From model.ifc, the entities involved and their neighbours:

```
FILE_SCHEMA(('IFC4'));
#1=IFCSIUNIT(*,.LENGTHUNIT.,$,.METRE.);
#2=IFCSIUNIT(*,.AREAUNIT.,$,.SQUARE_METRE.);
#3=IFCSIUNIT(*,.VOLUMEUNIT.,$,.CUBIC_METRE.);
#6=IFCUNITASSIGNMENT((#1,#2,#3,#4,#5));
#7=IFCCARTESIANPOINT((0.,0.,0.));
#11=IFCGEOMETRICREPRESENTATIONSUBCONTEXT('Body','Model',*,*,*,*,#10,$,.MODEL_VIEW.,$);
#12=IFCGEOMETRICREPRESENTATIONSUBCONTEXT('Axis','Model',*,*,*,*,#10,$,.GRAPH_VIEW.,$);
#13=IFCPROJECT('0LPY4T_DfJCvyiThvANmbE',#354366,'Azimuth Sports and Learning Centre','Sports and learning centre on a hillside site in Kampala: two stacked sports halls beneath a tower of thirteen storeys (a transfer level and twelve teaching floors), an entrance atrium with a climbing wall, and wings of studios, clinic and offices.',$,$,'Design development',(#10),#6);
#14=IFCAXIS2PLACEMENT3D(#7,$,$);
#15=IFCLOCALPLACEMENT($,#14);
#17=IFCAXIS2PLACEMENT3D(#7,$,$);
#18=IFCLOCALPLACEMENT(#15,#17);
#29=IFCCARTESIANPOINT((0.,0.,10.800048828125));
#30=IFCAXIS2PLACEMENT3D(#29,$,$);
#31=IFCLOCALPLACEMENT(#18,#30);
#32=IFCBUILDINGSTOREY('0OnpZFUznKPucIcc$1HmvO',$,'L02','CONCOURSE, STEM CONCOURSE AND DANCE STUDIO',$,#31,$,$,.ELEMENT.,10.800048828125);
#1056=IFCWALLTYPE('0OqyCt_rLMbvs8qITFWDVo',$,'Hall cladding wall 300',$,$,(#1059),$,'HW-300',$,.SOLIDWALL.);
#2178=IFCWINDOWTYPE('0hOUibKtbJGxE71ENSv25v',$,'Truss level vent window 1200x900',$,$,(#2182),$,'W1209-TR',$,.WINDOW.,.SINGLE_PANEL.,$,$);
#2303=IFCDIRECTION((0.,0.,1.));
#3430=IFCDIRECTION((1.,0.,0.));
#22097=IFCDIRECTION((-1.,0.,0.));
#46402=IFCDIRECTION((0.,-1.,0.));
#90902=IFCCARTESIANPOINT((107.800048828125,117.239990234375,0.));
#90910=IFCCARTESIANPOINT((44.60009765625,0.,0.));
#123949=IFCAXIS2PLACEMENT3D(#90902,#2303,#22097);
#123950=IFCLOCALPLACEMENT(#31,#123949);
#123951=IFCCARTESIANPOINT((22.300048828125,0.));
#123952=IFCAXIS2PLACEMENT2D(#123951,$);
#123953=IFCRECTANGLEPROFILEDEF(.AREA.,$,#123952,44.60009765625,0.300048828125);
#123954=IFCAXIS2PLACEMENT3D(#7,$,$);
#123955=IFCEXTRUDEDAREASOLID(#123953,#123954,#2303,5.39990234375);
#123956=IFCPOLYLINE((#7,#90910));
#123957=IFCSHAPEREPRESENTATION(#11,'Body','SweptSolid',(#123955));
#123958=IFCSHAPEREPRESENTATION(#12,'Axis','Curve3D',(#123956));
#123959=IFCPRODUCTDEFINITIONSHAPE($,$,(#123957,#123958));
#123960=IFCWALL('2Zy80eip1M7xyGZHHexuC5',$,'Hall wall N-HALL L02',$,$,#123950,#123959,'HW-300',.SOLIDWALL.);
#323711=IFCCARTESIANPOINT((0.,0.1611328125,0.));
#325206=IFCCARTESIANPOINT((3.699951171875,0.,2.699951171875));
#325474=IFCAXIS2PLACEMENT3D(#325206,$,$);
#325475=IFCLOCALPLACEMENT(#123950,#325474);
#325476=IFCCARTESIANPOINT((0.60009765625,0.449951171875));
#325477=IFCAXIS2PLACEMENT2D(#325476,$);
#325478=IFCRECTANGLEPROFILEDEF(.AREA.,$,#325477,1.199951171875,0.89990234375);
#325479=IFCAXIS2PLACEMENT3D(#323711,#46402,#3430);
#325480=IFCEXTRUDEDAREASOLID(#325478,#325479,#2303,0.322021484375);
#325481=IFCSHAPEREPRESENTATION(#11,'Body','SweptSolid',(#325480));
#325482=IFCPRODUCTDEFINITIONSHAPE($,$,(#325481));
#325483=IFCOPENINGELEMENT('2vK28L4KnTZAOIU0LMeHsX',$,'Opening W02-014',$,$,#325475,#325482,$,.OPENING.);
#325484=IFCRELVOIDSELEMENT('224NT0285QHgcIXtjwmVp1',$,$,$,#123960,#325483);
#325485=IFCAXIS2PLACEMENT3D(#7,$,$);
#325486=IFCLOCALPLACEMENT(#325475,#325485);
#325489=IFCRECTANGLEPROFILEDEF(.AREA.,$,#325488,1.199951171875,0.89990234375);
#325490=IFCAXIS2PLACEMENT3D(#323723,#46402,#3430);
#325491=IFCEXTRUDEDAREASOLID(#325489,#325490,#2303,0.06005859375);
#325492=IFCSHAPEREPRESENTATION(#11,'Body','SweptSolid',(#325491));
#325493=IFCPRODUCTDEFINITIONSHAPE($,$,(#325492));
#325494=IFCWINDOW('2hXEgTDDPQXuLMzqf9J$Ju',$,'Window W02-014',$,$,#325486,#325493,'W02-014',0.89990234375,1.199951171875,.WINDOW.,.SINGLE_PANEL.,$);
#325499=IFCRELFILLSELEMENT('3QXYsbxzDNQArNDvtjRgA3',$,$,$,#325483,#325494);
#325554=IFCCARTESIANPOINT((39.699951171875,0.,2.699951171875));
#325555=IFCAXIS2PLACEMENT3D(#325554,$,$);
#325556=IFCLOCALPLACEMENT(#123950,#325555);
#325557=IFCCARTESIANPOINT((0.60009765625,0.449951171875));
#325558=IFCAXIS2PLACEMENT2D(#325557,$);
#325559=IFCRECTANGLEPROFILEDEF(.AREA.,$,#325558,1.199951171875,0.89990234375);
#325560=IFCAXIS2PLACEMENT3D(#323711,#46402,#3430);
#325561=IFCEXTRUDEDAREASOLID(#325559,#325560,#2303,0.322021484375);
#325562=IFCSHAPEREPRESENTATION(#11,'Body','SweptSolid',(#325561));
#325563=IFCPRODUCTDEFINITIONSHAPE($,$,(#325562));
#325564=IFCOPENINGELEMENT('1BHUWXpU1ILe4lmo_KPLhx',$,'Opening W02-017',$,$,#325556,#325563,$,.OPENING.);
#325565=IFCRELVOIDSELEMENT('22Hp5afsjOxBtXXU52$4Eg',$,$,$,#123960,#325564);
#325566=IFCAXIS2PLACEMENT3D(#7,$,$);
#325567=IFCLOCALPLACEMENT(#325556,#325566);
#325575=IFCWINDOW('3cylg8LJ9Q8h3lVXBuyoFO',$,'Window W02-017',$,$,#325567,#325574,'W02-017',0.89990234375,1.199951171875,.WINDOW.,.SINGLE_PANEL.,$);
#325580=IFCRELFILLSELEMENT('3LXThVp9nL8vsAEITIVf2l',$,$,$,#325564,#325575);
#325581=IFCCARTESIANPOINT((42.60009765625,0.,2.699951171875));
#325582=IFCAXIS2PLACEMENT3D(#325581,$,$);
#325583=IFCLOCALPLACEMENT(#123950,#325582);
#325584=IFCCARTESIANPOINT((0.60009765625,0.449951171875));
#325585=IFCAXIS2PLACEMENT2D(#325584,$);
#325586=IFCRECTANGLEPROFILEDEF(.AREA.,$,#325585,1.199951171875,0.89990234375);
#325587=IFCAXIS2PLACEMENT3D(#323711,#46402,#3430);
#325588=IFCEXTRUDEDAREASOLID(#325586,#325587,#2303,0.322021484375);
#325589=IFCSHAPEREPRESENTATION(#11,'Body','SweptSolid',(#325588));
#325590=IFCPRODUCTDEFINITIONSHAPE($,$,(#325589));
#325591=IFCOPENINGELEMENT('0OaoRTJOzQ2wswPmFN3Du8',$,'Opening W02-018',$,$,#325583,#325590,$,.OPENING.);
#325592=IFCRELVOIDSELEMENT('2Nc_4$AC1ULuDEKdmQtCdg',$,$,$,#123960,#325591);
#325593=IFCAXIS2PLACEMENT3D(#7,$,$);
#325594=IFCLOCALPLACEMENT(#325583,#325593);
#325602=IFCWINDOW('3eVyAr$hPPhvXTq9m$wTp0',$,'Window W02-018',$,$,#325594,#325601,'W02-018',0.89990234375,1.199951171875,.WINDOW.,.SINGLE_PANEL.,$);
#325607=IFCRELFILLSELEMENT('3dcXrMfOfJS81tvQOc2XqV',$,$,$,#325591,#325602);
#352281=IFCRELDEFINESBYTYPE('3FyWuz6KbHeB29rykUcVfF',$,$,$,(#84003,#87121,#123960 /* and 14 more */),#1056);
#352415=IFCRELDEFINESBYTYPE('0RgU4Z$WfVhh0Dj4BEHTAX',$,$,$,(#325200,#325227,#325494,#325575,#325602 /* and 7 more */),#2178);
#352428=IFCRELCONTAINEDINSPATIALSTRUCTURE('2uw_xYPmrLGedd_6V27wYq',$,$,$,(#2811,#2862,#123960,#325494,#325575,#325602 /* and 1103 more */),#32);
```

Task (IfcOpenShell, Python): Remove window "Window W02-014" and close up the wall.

```python
import ifcopenshell
import ifcopenshell.api.feature
import ifcopenshell.api.root
import ifcopenshell.geom
import ifcopenshell.util.shape

model = ifcopenshell.open("model.ifc")
settings = ifcopenshell.geom.settings()


def volume(element):
    """Net volume in cubic metres, openings subtracted."""
    shape = ifcopenshell.geom.create_shape(settings, element)
    return ifcopenshell.util.shape.get_volume(shape.geometry)


window = model.by_guid("2hXEgTDDPQXuLMzqf9J$Ju")
opening = window.FillsVoids[0].RelatingOpeningElement
wall = opening.VoidsElements[0].RelatingBuildingElement
before = volume(wall)

ifcopenshell.api.root.remove_product(model, product=window)
ifcopenshell.api.feature.remove_feature(model, feature=opening)

after = volume(wall)

print(f"wall volume {before:.3f} -> {after:.3f} m3")

model.write("model_updated.ifc")
```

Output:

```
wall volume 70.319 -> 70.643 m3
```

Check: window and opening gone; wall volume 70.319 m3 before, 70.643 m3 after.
